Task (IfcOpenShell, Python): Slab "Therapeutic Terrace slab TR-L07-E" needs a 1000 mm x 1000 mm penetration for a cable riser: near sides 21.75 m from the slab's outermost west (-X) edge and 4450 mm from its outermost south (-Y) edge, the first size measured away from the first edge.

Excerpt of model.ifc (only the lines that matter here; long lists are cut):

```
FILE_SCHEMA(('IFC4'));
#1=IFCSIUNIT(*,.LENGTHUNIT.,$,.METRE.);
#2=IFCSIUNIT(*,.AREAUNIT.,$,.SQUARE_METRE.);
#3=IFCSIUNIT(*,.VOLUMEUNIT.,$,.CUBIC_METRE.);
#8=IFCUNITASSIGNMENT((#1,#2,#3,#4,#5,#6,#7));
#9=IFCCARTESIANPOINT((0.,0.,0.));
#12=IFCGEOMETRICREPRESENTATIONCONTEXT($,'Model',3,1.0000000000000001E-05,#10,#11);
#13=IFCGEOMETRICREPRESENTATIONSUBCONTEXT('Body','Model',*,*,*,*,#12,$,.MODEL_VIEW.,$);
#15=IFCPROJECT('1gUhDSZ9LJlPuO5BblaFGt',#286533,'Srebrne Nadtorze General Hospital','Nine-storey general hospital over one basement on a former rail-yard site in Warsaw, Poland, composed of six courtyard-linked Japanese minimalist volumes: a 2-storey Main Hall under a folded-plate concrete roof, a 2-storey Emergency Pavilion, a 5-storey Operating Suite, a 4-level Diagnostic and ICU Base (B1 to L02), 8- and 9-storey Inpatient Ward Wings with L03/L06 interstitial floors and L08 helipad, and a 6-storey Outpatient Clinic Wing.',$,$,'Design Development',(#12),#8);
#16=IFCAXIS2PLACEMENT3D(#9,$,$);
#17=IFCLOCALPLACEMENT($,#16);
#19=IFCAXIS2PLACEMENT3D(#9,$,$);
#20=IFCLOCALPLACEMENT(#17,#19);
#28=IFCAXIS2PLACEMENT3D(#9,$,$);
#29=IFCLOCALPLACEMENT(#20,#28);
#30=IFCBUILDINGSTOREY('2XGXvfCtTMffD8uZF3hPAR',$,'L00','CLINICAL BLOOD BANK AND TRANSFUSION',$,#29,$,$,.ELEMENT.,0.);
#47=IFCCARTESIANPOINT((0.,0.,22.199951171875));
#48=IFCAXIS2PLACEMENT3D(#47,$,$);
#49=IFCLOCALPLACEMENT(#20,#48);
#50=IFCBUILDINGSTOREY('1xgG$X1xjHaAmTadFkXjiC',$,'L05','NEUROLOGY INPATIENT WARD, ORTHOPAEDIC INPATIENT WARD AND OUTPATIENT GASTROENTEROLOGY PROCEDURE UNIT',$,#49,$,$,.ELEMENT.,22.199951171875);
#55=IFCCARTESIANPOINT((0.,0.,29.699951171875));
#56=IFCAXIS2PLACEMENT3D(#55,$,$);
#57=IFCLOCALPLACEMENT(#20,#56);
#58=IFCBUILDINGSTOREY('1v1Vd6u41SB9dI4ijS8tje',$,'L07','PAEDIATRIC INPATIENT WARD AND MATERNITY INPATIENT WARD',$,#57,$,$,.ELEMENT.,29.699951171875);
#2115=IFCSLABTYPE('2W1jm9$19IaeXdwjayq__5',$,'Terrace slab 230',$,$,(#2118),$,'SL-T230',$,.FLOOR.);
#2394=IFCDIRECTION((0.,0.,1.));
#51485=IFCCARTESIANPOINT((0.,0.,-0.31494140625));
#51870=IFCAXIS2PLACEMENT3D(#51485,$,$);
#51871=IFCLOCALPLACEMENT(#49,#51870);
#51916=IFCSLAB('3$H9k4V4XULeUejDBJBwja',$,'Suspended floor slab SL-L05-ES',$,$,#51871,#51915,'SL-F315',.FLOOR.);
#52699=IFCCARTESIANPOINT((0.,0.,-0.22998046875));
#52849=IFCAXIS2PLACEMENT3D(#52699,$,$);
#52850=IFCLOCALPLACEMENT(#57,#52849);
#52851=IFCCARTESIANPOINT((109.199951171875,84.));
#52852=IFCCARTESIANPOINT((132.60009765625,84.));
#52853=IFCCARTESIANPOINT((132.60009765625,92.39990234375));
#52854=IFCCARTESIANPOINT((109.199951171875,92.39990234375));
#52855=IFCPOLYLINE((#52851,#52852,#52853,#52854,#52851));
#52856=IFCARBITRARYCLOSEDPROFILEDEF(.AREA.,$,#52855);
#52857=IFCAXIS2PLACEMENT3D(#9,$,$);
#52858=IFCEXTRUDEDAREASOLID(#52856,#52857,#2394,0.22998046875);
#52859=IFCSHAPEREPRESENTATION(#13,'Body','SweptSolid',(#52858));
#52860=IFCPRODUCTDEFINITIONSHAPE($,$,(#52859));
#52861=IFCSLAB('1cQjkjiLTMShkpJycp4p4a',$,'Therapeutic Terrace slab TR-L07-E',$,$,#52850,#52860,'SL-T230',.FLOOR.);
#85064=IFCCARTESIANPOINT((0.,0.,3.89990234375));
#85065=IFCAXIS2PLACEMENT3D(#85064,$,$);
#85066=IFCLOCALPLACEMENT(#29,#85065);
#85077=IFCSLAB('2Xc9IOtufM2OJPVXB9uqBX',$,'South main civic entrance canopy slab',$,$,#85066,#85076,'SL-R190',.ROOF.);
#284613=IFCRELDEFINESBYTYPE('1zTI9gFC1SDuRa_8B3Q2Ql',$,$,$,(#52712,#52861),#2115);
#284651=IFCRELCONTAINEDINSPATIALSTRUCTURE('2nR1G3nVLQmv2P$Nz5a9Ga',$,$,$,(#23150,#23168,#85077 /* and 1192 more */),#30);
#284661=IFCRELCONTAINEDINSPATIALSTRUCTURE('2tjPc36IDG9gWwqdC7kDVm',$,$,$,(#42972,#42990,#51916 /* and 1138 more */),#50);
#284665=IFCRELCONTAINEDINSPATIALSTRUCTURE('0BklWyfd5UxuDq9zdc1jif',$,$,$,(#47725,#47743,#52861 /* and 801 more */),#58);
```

```python
import numpy as np
import ifcopenshell
import ifcopenshell.api.feature
import ifcopenshell.api.geometry
import ifcopenshell.api.root
import ifcopenshell.geom
import ifcopenshell.util.placement
import ifcopenshell.util.representation
import ifcopenshell.util.shape
import ifcopenshell.util.unit

model = ifcopenshell.open("model.ifc")
unit_scale = ifcopenshell.util.unit.calculate_unit_scale(model)
settings = ifcopenshell.geom.settings()


def volume(element):
    """Net volume in cubic metres, openings subtracted."""
    shape = ifcopenshell.geom.create_shape(settings, element)
    return ifcopenshell.util.shape.get_volume(shape.geometry)


slab = model.by_guid("1cQjkjiLTMShkpJycp4p4a")
before = volume(slab)

# Extent in the slab's own axes, in metres. The edges named are its -X and -Y sides.
slab_shape = ifcopenshell.geom.create_shape(settings, slab)
vertices = ifcopenshell.util.shape.get_vertices(slab_shape.geometry)
x_min, y_min, bottom = vertices.min(axis=0)
top = vertices[:, 2].max()

opening = ifcopenshell.api.root.create_entity(model, ifc_class="IfcOpeningElement", name="Cable riser opening", predefined_type="OPENING")
context = ifcopenshell.util.representation.get_context(model, "Model", "Body", "MODEL_VIEW")
width, depth = 1, 1
outline = [(0.0, 0.0), (width, 0.0), (width, depth), (0.0, depth), (0.0, 0.0)]
# Overshoot both faces by 50 mm so the cut is clean.
shape = ifcopenshell.api.geometry.add_slab_representation(
    model, context=context, depth=top - bottom + 0.1, polyline=outline
)
ifcopenshell.api.geometry.assign_representation(model, product=opening, representation=shape)

matrix = ifcopenshell.util.placement.get_local_placement(slab.ObjectPlacement)
matrix[:, 3] = matrix @ np.append(np.array([x_min + 21.75, y_min + 4.45, bottom - 0.05]) / unit_scale, 1.0)
ifcopenshell.api.geometry.edit_object_placement(model, product=opening, matrix=matrix, is_si=False)
ifcopenshell.api.feature.add_feature(model, feature=opening, element=slab)

after = volume(slab)

print(f"slab volume {before:.3f} -> {after:.3f} m3")

model.write("model_edited.ifc")
```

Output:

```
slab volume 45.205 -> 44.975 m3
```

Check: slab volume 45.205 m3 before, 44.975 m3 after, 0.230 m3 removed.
